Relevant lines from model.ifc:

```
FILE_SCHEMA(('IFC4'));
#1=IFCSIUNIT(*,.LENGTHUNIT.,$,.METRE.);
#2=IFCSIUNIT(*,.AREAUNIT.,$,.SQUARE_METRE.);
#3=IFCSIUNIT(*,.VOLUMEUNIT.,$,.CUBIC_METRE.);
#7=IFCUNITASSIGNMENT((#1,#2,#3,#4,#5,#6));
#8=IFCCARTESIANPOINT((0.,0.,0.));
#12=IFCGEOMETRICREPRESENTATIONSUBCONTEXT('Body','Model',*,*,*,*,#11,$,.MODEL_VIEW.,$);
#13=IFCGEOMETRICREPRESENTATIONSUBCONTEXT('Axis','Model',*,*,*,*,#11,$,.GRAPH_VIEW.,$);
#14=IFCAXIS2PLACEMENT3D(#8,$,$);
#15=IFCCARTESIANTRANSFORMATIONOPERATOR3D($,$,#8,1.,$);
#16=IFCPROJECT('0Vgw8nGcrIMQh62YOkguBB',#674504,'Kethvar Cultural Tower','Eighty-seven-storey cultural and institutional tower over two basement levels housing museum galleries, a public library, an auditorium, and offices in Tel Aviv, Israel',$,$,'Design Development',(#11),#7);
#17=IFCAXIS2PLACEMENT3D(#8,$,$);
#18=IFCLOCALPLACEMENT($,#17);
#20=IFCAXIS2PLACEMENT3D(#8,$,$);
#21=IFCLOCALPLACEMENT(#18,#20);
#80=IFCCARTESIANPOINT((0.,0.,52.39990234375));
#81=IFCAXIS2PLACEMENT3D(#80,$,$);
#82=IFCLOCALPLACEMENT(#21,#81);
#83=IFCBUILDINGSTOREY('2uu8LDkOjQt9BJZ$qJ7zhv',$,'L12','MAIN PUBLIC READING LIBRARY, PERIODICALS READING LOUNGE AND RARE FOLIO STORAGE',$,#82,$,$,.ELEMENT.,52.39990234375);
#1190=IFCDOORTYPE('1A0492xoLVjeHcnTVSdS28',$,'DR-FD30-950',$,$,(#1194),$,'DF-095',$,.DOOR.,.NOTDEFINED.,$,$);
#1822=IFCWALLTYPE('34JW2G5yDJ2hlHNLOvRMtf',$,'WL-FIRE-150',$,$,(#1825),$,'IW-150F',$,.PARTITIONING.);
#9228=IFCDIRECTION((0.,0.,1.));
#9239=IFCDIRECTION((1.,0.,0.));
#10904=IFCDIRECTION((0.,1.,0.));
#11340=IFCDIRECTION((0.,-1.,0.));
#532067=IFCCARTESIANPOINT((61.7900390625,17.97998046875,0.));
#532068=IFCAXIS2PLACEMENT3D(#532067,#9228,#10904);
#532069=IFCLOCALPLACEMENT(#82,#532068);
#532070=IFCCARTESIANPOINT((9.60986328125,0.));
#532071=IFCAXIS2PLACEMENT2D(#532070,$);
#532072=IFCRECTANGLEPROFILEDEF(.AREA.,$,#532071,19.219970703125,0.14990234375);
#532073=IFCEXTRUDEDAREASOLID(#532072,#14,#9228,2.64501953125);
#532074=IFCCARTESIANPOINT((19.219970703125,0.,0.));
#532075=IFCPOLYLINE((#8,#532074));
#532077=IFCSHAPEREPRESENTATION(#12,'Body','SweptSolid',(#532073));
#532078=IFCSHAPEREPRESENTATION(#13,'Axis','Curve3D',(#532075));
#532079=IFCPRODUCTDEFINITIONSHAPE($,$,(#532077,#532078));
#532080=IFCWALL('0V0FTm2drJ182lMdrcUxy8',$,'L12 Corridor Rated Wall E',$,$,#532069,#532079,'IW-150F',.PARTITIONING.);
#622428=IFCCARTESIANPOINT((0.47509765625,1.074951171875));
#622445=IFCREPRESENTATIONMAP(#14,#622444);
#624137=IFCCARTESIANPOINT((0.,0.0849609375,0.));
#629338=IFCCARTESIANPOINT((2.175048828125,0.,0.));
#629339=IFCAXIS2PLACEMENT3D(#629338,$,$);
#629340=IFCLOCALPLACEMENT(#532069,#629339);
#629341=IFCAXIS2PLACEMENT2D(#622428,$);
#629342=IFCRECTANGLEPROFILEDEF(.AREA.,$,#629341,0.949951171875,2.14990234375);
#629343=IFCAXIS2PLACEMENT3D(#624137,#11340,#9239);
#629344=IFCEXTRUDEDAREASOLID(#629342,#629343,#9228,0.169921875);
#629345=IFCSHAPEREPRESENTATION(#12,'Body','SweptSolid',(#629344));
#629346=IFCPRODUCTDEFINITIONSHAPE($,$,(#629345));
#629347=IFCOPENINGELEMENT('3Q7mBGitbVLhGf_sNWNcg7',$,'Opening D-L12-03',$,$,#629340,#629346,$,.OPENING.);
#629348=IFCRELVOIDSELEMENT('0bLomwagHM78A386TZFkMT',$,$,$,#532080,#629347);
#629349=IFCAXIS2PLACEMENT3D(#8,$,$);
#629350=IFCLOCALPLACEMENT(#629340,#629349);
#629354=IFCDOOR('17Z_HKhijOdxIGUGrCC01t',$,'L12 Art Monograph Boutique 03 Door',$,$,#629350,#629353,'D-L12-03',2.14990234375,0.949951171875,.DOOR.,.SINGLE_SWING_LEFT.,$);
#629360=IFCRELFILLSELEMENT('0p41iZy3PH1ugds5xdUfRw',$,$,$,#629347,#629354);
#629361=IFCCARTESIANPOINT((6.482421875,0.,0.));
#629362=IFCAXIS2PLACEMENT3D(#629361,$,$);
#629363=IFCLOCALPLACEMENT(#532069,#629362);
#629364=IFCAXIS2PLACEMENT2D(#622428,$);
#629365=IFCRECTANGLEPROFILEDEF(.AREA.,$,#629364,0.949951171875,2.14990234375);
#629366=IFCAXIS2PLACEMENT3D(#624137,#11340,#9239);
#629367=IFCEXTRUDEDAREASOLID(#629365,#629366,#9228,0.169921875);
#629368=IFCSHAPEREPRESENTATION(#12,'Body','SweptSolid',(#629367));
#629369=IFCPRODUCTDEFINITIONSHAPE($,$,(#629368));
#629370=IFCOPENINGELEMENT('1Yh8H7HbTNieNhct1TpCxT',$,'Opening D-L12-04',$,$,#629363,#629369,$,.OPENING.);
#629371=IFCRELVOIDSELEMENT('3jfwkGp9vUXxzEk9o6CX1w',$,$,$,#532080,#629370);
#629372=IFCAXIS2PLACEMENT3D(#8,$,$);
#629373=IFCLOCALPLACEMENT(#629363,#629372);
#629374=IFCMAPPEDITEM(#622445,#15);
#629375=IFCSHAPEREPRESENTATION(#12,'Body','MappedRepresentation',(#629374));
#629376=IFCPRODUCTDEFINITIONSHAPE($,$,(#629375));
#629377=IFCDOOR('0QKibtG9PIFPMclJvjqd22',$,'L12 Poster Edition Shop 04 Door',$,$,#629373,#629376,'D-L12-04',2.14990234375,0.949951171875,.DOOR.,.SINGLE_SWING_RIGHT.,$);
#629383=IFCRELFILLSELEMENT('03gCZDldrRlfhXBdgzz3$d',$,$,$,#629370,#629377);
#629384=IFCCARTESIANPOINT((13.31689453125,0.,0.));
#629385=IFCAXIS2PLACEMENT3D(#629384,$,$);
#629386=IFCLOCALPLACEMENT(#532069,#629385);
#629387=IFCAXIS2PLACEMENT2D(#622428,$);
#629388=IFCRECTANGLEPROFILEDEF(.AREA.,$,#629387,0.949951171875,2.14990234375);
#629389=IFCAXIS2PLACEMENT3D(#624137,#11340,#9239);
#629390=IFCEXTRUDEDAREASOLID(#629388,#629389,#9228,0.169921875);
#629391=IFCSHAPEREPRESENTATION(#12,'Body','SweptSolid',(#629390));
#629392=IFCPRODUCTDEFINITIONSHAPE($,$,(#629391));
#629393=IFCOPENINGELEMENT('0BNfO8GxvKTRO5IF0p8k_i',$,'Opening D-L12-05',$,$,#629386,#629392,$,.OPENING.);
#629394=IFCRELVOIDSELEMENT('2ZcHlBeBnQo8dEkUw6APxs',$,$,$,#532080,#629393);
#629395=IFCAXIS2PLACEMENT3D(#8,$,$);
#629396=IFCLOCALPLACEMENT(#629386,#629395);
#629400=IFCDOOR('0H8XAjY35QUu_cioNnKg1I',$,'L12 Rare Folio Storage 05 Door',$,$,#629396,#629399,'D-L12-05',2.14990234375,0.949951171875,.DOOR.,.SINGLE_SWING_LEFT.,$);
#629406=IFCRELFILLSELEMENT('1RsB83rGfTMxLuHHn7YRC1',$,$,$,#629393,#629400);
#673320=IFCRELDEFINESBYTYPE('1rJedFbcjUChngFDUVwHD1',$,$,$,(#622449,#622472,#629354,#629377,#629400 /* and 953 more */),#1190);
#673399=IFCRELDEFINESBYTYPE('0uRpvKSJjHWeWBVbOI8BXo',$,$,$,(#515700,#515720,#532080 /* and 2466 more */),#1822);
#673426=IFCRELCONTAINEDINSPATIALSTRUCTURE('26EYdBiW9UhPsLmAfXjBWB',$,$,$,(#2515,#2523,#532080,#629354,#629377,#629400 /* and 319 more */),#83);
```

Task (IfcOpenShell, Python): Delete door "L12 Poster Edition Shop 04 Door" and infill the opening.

```python
import ifcopenshell
import ifcopenshell.api.feature
import ifcopenshell.api.root
import ifcopenshell.geom
import ifcopenshell.util.shape

model = ifcopenshell.open("model.ifc")
settings = ifcopenshell.geom.settings()


def volume(element):
    """Net volume in cubic metres, openings subtracted."""
    shape = ifcopenshell.geom.create_shape(settings, element)
    return ifcopenshell.util.shape.get_volume(shape.geometry)


door = model.by_guid("0QKibtG9PIFPMclJvjqd22")
opening = door.FillsVoids[0].RelatingOpeningElement
wall = opening.VoidsElements[0].RelatingBuildingElement
before = volume(wall)

ifcopenshell.api.root.remove_product(model, product=door)
ifcopenshell.api.feature.remove_feature(model, feature=opening)

after = volume(wall)

print(f"wall volume {before:.3f} -> {after:.3f} m3")

model.write("model-out.ifc")
```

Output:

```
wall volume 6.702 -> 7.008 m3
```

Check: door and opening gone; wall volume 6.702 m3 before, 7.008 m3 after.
